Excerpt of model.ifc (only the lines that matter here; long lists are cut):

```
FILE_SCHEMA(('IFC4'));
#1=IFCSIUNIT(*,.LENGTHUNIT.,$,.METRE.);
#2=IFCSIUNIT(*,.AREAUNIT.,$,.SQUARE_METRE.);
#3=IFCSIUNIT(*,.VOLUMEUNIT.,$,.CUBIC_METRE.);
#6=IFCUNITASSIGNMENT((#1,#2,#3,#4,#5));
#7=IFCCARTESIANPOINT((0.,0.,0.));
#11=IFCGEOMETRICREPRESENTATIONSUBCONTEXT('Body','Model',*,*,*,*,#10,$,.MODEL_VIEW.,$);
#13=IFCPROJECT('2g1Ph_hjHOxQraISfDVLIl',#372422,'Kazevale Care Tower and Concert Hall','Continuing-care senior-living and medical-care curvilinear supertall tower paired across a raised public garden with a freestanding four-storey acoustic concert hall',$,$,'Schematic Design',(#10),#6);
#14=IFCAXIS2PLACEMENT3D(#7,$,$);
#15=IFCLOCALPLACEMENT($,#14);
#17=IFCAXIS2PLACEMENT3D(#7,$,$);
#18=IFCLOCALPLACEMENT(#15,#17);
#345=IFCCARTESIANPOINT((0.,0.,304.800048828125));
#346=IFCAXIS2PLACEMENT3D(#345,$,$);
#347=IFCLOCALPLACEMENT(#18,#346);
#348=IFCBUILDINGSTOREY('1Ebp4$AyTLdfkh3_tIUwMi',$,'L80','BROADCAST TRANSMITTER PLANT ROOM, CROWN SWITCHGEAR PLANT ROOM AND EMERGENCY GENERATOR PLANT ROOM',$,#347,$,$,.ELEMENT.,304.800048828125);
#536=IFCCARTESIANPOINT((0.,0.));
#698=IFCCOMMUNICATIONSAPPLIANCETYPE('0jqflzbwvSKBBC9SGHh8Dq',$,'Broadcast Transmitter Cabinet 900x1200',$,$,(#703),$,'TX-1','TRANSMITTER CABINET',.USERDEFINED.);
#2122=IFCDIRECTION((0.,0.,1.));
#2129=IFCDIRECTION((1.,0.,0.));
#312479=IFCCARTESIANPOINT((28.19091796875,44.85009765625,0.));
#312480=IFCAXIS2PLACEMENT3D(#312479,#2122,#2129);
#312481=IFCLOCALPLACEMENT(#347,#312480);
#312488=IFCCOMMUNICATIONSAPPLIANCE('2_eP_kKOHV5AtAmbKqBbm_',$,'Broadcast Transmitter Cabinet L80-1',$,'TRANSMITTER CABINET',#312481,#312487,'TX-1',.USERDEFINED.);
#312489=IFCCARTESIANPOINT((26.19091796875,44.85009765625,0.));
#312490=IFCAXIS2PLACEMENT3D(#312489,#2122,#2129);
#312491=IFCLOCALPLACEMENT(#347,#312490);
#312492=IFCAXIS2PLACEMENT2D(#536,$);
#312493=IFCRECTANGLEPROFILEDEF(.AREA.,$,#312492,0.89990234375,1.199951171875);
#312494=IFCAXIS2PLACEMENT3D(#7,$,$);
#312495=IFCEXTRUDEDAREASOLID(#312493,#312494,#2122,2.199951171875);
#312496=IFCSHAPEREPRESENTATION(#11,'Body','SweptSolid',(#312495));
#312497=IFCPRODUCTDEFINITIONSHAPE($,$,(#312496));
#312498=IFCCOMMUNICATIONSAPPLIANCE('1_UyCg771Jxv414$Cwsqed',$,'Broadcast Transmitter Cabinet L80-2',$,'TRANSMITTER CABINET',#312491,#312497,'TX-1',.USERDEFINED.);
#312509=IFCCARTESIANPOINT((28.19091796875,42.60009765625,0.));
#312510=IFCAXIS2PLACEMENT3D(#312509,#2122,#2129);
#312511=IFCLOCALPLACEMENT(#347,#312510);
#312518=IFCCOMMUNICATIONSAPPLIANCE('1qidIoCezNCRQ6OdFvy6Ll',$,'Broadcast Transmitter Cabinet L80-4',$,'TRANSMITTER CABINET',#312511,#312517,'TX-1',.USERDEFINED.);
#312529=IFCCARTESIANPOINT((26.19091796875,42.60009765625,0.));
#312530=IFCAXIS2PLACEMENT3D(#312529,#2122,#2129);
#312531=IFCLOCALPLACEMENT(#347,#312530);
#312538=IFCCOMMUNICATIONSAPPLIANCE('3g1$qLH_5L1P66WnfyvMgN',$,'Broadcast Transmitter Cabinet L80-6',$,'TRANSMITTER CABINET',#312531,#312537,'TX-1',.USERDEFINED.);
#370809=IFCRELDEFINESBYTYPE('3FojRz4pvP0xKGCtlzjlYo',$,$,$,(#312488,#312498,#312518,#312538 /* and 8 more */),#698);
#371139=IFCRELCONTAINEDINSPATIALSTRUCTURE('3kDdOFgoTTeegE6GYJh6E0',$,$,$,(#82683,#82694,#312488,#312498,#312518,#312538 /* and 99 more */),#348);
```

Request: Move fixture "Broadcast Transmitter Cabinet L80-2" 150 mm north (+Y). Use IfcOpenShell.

```python
import ifcopenshell
import ifcopenshell.api.geometry
import ifcopenshell.util.placement

model = ifcopenshell.open("model.ifc")

item = model.by_guid("1_UyCg771Jxv414$Cwsqed")
matrix = ifcopenshell.util.placement.get_local_placement(item.ObjectPlacement)
matrix[1, 3] += 0.15
ifcopenshell.api.geometry.edit_object_placement(model, product=item, matrix=matrix, is_si=False)

print(ifcopenshell.util.placement.get_local_placement(item.ObjectPlacement).round(3) + 0.0)

model.write("model-out.ifc")
```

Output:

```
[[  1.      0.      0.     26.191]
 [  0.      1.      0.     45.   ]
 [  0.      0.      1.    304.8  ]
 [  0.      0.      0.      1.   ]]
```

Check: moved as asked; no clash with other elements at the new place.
